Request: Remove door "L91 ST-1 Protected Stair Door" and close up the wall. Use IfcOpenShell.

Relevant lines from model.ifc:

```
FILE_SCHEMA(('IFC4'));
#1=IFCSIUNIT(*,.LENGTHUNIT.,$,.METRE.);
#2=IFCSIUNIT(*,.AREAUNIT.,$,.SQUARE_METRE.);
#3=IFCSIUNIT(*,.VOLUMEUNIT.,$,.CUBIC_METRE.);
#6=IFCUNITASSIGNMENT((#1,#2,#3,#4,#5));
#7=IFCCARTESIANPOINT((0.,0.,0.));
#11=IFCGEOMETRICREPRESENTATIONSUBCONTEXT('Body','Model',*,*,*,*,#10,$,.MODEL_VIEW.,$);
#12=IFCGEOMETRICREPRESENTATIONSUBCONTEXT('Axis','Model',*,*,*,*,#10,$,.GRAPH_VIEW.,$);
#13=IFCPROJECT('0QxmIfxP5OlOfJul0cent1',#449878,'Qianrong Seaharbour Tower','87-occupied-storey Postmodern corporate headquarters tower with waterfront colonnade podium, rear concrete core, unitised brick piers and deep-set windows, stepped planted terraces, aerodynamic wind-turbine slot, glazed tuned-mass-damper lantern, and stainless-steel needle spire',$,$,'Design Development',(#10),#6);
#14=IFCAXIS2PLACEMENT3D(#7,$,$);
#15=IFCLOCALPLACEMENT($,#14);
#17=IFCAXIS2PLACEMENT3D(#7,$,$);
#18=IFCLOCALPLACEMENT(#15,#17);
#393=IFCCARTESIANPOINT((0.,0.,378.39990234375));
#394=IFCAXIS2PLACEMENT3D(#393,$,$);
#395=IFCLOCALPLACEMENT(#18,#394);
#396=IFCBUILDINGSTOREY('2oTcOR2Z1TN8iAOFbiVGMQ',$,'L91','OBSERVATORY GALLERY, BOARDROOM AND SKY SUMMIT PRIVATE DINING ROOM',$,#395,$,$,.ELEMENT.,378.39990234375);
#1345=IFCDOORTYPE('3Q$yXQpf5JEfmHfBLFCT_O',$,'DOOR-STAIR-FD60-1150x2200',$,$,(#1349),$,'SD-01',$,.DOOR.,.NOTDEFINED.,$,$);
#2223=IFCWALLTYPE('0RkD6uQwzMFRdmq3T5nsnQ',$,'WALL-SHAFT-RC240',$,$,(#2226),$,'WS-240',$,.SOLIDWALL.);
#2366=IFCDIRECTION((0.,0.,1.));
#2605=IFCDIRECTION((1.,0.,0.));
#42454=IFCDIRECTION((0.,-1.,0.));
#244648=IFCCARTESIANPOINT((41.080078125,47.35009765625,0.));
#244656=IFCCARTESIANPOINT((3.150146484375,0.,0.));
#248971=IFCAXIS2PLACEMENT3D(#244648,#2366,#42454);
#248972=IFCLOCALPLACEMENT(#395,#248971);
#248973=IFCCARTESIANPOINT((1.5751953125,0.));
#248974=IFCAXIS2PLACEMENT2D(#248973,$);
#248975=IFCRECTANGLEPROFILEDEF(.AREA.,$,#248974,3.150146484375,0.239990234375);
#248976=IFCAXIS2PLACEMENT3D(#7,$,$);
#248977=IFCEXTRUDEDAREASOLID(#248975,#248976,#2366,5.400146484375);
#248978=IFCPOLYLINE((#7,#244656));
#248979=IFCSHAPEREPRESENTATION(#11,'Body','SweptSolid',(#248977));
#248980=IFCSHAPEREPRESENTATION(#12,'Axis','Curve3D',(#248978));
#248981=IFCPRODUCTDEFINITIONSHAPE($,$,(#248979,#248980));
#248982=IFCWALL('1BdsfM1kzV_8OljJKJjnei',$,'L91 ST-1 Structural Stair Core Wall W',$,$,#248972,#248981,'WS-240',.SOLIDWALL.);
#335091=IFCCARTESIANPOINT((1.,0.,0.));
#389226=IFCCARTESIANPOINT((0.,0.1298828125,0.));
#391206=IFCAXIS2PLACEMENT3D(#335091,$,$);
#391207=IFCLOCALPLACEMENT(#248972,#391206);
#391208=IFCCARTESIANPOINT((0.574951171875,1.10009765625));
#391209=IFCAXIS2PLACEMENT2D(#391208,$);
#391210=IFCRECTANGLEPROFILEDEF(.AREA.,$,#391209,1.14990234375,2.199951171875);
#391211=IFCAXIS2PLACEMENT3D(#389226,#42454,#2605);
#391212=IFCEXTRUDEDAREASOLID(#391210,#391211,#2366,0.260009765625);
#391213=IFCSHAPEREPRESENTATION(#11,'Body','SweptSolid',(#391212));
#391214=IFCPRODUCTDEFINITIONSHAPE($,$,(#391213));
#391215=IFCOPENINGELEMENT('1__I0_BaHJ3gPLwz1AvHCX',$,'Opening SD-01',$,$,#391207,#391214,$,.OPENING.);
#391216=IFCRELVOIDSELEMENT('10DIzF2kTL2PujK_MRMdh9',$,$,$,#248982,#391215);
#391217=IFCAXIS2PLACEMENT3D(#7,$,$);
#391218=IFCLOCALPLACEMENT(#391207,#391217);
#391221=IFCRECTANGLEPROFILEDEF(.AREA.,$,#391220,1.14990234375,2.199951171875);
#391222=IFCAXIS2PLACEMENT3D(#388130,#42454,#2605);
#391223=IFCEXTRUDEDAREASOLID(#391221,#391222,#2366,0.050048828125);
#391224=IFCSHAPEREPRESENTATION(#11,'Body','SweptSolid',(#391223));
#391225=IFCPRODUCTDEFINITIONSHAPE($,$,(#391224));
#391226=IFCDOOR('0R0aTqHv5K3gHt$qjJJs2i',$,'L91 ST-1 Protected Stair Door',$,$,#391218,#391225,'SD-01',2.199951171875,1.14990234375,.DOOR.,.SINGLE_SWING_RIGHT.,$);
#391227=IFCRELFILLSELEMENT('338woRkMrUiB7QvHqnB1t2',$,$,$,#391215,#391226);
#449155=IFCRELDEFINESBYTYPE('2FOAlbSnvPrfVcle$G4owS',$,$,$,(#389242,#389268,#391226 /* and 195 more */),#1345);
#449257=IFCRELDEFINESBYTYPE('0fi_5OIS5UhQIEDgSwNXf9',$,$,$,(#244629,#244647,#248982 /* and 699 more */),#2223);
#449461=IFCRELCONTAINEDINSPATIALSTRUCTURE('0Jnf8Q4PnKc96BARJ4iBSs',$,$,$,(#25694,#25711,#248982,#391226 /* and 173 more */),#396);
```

```python
import ifcopenshell
import ifcopenshell.api.feature
import ifcopenshell.api.root
import ifcopenshell.geom
import ifcopenshell.util.shape

model = ifcopenshell.open("model.ifc")
settings = ifcopenshell.geom.settings()


def volume(element):
    """Net volume in cubic metres, openings subtracted."""
    shape = ifcopenshell.geom.create_shape(settings, element)
    return ifcopenshell.util.shape.get_volume(shape.geometry)


door = model.by_guid("0R0aTqHv5K3gHt$qjJJs2i")
opening = door.FillsVoids[0].RelatingOpeningElement
wall = opening.VoidsElements[0].RelatingBuildingElement
before = volume(wall)

ifcopenshell.api.root.remove_product(model, product=door)
ifcopenshell.api.feature.remove_feature(model, feature=opening)

after = volume(wall)

print(f"wall volume {before:.3f} -> {after:.3f} m3")

model.write("model_edited.ifc")
```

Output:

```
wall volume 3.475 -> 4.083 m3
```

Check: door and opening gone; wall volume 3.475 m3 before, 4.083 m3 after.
